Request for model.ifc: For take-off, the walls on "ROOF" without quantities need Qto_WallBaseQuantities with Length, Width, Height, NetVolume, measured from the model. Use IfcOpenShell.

First a look at what the model holds.

```python
import ifcopenshell
import ifcopenshell.util.element
import ifcopenshell.util.unit

model = ifcopenshell.open("model.ifc")
print(model.schema)
for unit_type in ("LENGTHUNIT", "AREAUNIT", "VOLUMEUNIT"):
    print(unit_type, ifcopenshell.util.unit.calculate_unit_scale(model, unit_type))
storey = next(s for s in model.by_type("IfcBuildingStorey") if s.Name == "ROOF")
walls = [e for e in ifcopenshell.util.element.get_decomposition(storey) if e.is_a("IfcWall")]
for e in sorted(walls, key=lambda e: e.id()):
    print(e.id(), e.is_a(), e.Name, list(ifcopenshell.util.element.get_psets(e, qtos_only=True)), sep=" | ")
```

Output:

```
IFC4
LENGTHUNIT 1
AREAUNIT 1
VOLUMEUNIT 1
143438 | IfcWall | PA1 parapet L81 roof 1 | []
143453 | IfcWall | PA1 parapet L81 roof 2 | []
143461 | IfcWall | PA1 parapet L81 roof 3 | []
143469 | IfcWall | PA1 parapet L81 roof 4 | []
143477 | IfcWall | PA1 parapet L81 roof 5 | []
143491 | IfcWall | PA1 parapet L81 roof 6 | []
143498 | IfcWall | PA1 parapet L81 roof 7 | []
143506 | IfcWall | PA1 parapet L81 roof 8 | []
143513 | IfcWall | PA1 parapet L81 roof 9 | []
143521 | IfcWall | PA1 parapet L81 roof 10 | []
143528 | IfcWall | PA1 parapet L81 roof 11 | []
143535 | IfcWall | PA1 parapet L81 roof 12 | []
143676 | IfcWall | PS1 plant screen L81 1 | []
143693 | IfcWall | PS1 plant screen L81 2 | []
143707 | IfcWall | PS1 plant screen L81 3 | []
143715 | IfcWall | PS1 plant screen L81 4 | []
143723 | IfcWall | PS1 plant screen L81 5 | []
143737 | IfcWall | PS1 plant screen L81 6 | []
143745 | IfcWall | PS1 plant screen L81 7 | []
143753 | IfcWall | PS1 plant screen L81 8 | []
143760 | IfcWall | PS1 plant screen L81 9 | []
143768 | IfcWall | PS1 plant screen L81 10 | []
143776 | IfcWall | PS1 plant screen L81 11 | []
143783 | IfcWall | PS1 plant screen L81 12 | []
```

```python
import ifcopenshell
import ifcopenshell.api.pset
import ifcopenshell.geom
import ifcopenshell.util.element
import ifcopenshell.util.shape
import ifcopenshell.util.unit

model = ifcopenshell.open("model.ifc")
unit_scale = ifcopenshell.util.unit.calculate_unit_scale(model)
volume_scale = ifcopenshell.util.unit.calculate_unit_scale(model, "VOLUMEUNIT")
settings = ifcopenshell.geom.settings()

storey = next(s for s in model.by_type("IfcBuildingStorey") if s.Name == "ROOF")
walls = [e for e in ifcopenshell.util.element.get_decomposition(storey) if e.is_a("IfcWall")]

for e in sorted(walls, key=lambda e: e.id()):
    if ifcopenshell.util.element.get_psets(e, qtos_only=True, should_inherit=False):
        continue
    # Geometry comes back in metres, in the element's own axes.
    shape = ifcopenshell.geom.create_shape(settings, e)
    values = {
        "Length": ifcopenshell.util.shape.get_x(shape.geometry) / unit_scale,
        "Width": ifcopenshell.util.shape.get_y(shape.geometry) / unit_scale,
        "Height": ifcopenshell.util.shape.get_z(shape.geometry) / unit_scale,
        "NetVolume": ifcopenshell.util.shape.get_volume(shape.geometry) / volume_scale,
    }
    qto = ifcopenshell.api.pset.add_qto(model, product=e, name="Qto_WallBaseQuantities")
    ifcopenshell.api.pset.edit_qto(model, qto=qto, properties=values)
    print(e.id(), {k: round(v, 3) for k, v in values.items()})

model.write("model_rev.ifc")
```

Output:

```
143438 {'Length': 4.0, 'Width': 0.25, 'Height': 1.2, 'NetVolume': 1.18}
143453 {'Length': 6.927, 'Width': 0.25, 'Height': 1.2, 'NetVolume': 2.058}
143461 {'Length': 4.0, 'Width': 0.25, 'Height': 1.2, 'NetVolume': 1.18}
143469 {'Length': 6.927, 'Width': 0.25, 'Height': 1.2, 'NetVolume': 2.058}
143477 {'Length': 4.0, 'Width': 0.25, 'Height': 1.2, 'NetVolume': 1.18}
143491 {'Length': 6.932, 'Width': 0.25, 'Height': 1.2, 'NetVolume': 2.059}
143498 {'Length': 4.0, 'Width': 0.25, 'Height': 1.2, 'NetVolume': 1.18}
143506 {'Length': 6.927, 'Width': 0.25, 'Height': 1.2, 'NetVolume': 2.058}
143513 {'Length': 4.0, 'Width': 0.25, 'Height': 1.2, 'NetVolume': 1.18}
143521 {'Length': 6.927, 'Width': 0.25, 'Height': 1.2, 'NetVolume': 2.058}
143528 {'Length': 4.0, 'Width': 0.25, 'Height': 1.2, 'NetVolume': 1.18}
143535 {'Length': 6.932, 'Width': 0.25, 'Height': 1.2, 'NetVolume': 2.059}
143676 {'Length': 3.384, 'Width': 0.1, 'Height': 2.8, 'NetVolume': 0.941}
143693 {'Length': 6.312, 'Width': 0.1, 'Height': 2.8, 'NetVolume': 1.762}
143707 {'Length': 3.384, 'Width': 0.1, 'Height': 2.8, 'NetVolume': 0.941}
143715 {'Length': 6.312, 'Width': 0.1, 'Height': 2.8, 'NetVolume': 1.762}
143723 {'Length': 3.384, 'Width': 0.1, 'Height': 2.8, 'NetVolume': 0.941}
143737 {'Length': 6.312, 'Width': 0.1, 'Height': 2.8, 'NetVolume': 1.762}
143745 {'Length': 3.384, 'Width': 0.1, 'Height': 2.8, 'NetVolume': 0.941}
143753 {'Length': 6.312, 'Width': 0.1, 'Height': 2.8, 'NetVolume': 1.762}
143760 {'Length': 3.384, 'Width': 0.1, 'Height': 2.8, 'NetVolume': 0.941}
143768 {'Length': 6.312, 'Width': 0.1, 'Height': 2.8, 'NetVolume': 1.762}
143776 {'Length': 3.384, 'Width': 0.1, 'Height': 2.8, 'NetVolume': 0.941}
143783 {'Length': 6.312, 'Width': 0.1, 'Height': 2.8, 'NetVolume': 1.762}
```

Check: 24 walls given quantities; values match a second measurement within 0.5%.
